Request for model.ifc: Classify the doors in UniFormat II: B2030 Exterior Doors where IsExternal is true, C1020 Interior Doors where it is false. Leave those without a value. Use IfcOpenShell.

First a look at what the model holds.

```python
import ifcopenshell
import ifcopenshell.util.element

model = ifcopenshell.open("model.ifc")
print(model.schema)
print("classifications:", [c.Name for c in model.by_type("IfcClassification")])
values = [ifcopenshell.util.element.get_pset(e, "Pset_DoorCommon", "IsExternal") for e in model.by_type("IfcDoor")]
for value in (True, False, None):
    print("IsExternal", value, values.count(value))
```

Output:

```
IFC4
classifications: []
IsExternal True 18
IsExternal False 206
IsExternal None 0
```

```python
import ifcopenshell
import ifcopenshell.api.classification
import ifcopenshell.util.element

model = ifcopenshell.open("model.ifc")

system = ifcopenshell.api.classification.add_classification(model, classification="UniFormat II")

doors = model.by_type("IfcDoor")
external = {e: ifcopenshell.util.element.get_pset(e, "Pset_DoorCommon", "IsExternal") for e in doors}
for flag, code, name in ((True, "B2030", "Exterior Doors"), (False, "C1020", "Interior Doors")):
    products = [e for e in doors if external[e] is flag]
    ifcopenshell.api.classification.add_reference(
        model, products=products, classification=system, identification=code, name=name
    )
    print(code, len(products))

model.write("model_rev.ifc")
```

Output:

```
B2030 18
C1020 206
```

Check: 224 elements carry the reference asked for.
